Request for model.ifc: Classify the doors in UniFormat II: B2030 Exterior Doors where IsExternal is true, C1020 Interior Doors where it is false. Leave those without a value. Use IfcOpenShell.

First a look at what the model holds.

```python
import ifcopenshell
import ifcopenshell.util.element

model = ifcopenshell.open("model.ifc")
print(model.schema)
print("classifications:", [c.Name for c in model.by_type("IfcClassification")])
values = [ifcopenshell.util.element.get_pset(e, "Pset_DoorCommon", "IsExternal") for e in model.by_type("IfcDoor")]
for value in (True, False, None):
    print("IsExternal", value, values.count(value))
```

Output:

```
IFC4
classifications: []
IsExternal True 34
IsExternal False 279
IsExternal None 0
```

```python
import ifcopenshell
import ifcopenshell.api.classification
import ifcopenshell.util.element

model = ifcopenshell.open("model.ifc")

system = ifcopenshell.api.classification.add_classification(model, classification="UniFormat II")

doors = model.by_type("IfcDoor")
external = {e: ifcopenshell.util.element.get_pset(e, "Pset_DoorCommon", "IsExternal") for e in doors}
for flag, code, name in ((True, "B2030", "Exterior Doors"), (False, "C1020", "Interior Doors")):
    products = [e for e in doors if external[e] is flag]
    ifcopenshell.api.classification.add_reference(
        model, products=products, classification=system, identification=code, name=name
    )
    print(code, len(products))

model.write("model-out.ifc")
```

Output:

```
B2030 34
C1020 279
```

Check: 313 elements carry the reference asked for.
